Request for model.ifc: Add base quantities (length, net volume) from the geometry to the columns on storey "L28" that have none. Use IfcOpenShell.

First a look at what the model holds.

```python
import ifcopenshell
import ifcopenshell.util.element
import ifcopenshell.util.unit

model = ifcopenshell.open("model.ifc")
print(model.schema)
for unit_type in ("LENGTHUNIT", "AREAUNIT", "VOLUMEUNIT"):
    print(unit_type, ifcopenshell.util.unit.calculate_unit_scale(model, unit_type))
storey = next(s for s in model.by_type("IfcBuildingStorey") if s.Name == "L28")
columns = [e for e in ifcopenshell.util.element.get_decomposition(storey) if e.is_a("IfcColumn")]
for e in sorted(columns, key=lambda e: e.id()):
    print(e.id(), e.is_a(), e.Name, list(ifcopenshell.util.element.get_psets(e, qtos_only=True)), sep=" | ")
```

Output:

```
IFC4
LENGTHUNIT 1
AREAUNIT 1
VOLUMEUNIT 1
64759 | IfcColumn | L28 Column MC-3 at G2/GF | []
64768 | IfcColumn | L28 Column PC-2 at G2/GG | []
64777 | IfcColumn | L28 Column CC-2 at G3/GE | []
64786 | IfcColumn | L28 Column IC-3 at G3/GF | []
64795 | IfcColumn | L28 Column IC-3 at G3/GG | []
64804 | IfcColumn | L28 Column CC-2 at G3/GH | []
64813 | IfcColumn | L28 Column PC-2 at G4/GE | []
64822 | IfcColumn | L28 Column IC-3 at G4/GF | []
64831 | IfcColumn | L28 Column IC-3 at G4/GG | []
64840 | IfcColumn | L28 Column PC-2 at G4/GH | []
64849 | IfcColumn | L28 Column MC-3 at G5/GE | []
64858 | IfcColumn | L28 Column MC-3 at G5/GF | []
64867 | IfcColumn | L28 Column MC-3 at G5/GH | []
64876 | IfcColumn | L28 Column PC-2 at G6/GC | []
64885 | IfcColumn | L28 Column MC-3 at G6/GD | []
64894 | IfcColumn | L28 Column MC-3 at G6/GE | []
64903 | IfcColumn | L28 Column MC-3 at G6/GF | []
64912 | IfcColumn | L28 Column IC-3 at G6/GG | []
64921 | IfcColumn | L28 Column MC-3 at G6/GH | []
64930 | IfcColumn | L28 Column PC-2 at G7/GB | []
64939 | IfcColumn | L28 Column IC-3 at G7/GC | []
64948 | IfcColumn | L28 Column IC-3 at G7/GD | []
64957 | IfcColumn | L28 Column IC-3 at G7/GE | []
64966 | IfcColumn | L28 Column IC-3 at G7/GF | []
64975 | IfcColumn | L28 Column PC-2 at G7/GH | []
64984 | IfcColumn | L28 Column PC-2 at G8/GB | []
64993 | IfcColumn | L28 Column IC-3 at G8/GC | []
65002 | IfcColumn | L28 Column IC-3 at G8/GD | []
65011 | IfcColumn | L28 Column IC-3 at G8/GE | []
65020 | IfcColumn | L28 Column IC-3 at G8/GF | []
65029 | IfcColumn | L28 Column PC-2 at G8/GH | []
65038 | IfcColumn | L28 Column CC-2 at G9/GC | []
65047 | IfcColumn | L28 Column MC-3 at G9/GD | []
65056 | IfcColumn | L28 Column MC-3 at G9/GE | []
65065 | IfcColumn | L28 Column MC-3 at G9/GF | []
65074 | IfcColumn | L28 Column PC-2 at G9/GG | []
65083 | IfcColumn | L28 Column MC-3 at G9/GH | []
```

```python
import ifcopenshell
import ifcopenshell.api.pset
import ifcopenshell.geom
import ifcopenshell.util.element
import ifcopenshell.util.shape
import ifcopenshell.util.unit

model = ifcopenshell.open("model.ifc")
unit_scale = ifcopenshell.util.unit.calculate_unit_scale(model)
volume_scale = ifcopenshell.util.unit.calculate_unit_scale(model, "VOLUMEUNIT")
settings = ifcopenshell.geom.settings()

storey = next(s for s in model.by_type("IfcBuildingStorey") if s.Name == "L28")
columns = [e for e in ifcopenshell.util.element.get_decomposition(storey) if e.is_a("IfcColumn")]

for e in sorted(columns, key=lambda e: e.id()):
    if ifcopenshell.util.element.get_psets(e, qtos_only=True, should_inherit=False):
        continue
    # Geometry comes back in metres, in the element's own axes.
    shape = ifcopenshell.geom.create_shape(settings, e)
    values = {
        "Length": ifcopenshell.util.shape.get_z(shape.geometry) / unit_scale,
        "NetVolume": ifcopenshell.util.shape.get_volume(shape.geometry) / volume_scale,
    }
    qto = ifcopenshell.api.pset.add_qto(model, product=e, name="Qto_ColumnBaseQuantities")
    ifcopenshell.api.pset.edit_qto(model, qto=qto, properties=values)
    print(e.id(), {k: round(v, 3) for k, v in values.items()})

model.write("model_v2.ifc")
```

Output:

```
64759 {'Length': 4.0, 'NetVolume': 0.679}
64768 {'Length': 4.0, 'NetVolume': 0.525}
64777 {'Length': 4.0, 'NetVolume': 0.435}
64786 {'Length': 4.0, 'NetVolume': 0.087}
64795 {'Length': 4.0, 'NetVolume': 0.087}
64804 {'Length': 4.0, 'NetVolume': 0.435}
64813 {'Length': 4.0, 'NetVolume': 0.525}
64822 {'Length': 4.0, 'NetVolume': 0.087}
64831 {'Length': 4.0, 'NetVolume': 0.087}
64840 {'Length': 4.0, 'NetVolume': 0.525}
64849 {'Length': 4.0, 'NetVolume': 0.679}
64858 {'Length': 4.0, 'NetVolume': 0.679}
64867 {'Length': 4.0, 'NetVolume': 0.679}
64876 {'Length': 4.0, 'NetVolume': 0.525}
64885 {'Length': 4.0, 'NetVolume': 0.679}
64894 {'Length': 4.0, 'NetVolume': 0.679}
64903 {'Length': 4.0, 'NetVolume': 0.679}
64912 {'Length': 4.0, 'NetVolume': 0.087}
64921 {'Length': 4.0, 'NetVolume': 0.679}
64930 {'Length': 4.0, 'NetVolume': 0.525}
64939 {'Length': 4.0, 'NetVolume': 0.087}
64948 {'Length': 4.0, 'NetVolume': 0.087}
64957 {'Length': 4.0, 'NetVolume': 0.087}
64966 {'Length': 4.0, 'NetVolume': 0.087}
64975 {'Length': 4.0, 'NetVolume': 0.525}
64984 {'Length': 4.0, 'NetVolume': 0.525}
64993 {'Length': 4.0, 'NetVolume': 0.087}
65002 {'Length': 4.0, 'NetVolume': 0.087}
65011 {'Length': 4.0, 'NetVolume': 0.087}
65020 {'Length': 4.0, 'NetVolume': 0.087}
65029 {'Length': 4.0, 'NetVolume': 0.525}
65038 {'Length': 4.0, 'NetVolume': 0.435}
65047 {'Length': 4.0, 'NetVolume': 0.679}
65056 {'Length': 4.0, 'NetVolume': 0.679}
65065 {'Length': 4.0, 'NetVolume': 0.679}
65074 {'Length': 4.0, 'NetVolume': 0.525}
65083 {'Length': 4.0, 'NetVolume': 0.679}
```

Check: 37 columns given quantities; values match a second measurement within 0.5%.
